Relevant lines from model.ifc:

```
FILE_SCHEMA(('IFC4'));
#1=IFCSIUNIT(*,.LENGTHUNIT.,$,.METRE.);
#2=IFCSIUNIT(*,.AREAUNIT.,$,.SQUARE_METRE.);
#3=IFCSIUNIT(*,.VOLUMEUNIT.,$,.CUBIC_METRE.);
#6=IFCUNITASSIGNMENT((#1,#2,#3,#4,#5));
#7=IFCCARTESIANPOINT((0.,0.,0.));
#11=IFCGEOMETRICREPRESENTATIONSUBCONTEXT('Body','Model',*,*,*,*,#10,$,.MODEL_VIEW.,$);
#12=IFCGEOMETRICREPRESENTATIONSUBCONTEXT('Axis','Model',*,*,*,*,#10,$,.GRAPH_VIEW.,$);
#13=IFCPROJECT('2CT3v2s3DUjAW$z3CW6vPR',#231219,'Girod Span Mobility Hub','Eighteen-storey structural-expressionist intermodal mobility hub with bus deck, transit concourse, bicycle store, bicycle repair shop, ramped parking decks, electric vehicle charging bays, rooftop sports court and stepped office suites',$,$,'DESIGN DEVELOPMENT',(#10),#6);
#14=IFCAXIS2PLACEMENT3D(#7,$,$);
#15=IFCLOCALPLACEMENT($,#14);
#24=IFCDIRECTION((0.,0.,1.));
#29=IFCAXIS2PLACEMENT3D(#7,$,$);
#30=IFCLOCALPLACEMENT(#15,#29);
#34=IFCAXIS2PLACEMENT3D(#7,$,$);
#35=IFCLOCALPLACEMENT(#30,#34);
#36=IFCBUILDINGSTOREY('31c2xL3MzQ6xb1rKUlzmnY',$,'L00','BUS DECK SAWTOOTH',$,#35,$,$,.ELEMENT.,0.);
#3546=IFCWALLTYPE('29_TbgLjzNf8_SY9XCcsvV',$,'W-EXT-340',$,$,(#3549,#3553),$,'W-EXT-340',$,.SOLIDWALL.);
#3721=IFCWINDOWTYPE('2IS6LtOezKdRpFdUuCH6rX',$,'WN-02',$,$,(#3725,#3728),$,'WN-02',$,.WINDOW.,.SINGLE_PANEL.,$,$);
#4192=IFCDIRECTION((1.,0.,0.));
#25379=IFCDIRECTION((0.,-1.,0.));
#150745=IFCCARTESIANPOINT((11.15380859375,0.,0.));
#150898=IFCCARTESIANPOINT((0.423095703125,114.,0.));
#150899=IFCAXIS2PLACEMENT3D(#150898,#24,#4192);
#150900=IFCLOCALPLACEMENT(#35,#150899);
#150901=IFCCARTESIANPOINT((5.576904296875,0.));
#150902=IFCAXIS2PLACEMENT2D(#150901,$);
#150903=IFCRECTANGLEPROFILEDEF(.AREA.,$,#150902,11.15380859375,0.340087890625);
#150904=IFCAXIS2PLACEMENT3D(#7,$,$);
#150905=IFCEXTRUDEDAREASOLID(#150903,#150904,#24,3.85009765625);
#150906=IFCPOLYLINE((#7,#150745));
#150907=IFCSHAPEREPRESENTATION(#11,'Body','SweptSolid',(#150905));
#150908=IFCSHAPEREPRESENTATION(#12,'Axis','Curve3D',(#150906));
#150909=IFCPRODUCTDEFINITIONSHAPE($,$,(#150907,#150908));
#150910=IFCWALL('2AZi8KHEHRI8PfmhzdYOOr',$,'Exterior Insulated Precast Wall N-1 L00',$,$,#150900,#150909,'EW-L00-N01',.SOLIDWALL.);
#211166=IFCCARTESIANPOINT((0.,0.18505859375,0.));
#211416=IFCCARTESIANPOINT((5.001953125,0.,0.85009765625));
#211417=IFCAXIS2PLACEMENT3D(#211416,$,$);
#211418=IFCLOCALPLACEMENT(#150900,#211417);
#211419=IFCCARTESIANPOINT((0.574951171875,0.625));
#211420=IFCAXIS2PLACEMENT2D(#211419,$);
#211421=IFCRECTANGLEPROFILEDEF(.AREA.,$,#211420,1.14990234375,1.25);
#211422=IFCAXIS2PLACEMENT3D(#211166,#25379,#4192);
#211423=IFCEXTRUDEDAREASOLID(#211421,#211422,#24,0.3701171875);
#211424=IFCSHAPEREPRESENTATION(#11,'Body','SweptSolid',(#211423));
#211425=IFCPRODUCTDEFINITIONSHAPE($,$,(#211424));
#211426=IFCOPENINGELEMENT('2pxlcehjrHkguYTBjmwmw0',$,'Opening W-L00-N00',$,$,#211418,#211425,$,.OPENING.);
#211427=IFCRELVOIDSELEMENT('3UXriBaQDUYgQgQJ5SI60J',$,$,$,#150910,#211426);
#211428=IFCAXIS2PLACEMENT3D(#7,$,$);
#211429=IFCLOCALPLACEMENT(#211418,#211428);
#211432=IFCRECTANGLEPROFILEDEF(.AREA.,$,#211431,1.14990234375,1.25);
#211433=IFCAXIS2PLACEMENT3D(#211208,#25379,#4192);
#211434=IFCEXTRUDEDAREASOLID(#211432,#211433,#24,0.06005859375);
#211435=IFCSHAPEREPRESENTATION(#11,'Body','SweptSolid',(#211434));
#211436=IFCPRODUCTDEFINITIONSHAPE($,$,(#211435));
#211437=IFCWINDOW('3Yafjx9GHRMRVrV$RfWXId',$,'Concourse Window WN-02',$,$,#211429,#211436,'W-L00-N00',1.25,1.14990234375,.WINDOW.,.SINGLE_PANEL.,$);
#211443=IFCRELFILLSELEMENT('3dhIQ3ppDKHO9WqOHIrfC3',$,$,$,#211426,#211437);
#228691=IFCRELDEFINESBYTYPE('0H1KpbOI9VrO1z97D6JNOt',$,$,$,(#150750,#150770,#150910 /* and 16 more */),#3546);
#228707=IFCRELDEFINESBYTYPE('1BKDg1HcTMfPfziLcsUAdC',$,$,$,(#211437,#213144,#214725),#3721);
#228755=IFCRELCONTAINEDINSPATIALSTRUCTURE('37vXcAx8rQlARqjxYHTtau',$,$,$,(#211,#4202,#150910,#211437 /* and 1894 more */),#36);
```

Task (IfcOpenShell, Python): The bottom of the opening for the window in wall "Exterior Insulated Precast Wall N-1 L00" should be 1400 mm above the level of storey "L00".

```python
import numpy as np
import ifcopenshell
import ifcopenshell.api.geometry
import ifcopenshell.geom
import ifcopenshell.util.element
import ifcopenshell.util.placement
import ifcopenshell.util.shape
import ifcopenshell.util.unit

model = ifcopenshell.open("model.ifc")
unit_scale = ifcopenshell.util.unit.calculate_unit_scale(model)

window = model.by_id(211437)
opening = window.FillsVoids[0].RelatingOpeningElement
storey = ifcopenshell.util.element.get_container(window, ifc_class="IfcBuildingStorey")
level = ifcopenshell.util.placement.get_local_placement(storey.ObjectPlacement)[2, 3]

# The opening's origin need not be at the sill, so measure its lowest point.
shape = ifcopenshell.geom.create_shape(ifcopenshell.geom.settings(), opening)
bottom = ifcopenshell.util.shape.get_shape_bottom_elevation(shape, shape.geometry) / unit_scale
dz = level + 1.4 - bottom

shift = np.array([0.0, 0.0, dz])
# The window is placed relative to its opening, so it follows when the opening moves.
matrix = ifcopenshell.util.placement.get_local_placement(opening.ObjectPlacement)
matrix[:3, 3] += shift
ifcopenshell.api.geometry.edit_object_placement(
    model, product=opening, matrix=matrix, is_si=False, should_transform_children=True
)

print(f"moved by {dz * unit_scale:+.3f} m")

model.write("model_updated.ifc")
```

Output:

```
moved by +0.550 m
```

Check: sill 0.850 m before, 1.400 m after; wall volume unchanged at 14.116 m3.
